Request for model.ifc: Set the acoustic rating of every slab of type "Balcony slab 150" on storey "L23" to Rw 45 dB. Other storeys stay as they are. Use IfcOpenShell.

First a look at what the model holds.

```python
import ifcopenshell
import ifcopenshell.util.element

model = ifcopenshell.open("model.ifc")
print(model.schema)
storey = next(s for s in model.by_type("IfcBuildingStorey") if s.Name == "L23")
slabs = [e for e in ifcopenshell.util.element.get_decomposition(storey) if e.is_a("IfcSlab")]
seen = {}
for e in slabs:
    element_type = ifcopenshell.util.element.get_type(e)
    key = (element_type.Name if element_type != e and element_type else None, ifcopenshell.util.element.get_pset(e, "Pset_SlabCommon", "AcousticRating"))
    seen[key] = seen.get(key, 0) + 1
for (name, value), count in sorted(seen.items(), key=str):
    print(count, "x", name, "|", value)
```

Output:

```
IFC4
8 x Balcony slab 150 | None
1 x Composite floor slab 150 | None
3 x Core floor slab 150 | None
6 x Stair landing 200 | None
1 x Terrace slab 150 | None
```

```python
import ifcopenshell
import ifcopenshell.api.pset
import ifcopenshell.util.element

model = ifcopenshell.open("model.ifc")

storey = next(s for s in model.by_type("IfcBuildingStorey") if s.Name == "L23")
slabs = [e for e in ifcopenshell.util.element.get_decomposition(storey) if e.is_a("IfcSlab")]

count = 0
for e in slabs:
    element_type = ifcopenshell.util.element.get_type(e)
    if element_type in (None, e) or element_type.Name != "Balcony slab 150":
        continue
    # add_pset returns the element's existing set when there is one.
    pset = ifcopenshell.api.pset.add_pset(model, product=e, name="Pset_SlabCommon")
    ifcopenshell.api.pset.edit_pset(model, pset=pset, properties={"AcousticRating": "Rw 45 dB"})
    count += 1

print(count, "slabs updated")

model.write("model_v2.ifc")
```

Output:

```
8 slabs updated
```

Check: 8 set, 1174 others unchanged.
